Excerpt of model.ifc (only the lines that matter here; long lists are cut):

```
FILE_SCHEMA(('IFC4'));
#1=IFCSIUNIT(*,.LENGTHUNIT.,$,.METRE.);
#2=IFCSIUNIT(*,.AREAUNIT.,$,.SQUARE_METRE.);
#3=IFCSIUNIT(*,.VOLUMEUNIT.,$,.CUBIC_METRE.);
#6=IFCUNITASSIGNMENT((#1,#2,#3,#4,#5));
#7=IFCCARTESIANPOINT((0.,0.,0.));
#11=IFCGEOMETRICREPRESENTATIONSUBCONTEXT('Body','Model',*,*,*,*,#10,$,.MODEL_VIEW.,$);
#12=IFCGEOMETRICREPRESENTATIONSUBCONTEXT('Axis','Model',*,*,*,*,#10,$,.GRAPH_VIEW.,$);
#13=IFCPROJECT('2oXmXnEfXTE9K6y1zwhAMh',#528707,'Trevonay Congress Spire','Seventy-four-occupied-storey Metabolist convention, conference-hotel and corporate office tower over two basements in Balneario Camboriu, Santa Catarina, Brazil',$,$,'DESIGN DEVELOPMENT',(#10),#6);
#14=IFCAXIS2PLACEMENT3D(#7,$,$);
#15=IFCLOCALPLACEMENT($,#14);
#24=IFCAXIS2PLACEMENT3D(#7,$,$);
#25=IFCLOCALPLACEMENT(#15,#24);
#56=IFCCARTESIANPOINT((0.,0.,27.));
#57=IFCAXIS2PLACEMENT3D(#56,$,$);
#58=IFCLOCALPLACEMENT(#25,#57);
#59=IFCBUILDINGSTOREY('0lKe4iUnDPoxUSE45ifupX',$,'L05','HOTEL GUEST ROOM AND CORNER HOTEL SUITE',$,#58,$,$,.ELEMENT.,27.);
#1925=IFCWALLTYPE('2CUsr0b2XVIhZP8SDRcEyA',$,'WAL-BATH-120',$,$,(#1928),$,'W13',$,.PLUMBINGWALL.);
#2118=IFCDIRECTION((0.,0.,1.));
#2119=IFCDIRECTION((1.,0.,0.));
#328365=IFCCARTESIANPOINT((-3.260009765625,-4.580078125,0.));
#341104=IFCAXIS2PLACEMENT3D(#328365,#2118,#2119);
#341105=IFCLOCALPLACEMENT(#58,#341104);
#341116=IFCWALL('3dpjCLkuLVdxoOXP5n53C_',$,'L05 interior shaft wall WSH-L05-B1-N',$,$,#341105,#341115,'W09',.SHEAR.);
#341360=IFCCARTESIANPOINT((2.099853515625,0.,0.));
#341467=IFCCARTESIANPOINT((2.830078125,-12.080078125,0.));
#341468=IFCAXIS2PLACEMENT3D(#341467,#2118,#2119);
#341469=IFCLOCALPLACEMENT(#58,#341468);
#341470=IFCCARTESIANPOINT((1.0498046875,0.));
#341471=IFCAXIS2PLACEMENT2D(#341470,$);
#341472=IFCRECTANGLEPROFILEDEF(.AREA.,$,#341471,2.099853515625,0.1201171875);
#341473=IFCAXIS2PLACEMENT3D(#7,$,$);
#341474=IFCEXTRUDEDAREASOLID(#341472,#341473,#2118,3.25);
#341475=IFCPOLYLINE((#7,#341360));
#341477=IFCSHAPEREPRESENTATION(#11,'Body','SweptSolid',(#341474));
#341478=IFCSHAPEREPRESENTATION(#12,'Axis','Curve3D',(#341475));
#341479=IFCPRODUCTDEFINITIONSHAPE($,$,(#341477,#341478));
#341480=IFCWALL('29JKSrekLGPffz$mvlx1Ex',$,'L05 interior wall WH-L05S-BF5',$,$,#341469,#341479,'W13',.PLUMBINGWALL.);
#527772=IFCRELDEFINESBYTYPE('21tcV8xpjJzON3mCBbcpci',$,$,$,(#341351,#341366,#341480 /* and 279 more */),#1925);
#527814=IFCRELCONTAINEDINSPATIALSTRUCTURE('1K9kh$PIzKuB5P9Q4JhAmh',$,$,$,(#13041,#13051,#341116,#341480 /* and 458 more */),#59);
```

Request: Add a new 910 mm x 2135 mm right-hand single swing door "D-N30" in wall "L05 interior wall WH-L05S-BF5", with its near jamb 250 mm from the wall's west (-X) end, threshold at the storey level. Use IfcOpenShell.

```python
import numpy as np
import ifcopenshell
import ifcopenshell.api.feature
import ifcopenshell.api.geometry
import ifcopenshell.api.root
import ifcopenshell.api.spatial
import ifcopenshell.geom
import ifcopenshell.util.element
import ifcopenshell.util.placement
import ifcopenshell.util.representation
import ifcopenshell.util.shape
import ifcopenshell.util.unit

model = ifcopenshell.open("model.ifc")
unit_scale = ifcopenshell.util.unit.calculate_unit_scale(model)
settings = ifcopenshell.geom.settings()


def volume(element):
    """Net volume in cubic metres, openings subtracted."""
    shape = ifcopenshell.geom.create_shape(settings, element)
    return ifcopenshell.util.shape.get_volume(shape.geometry)


wall = model.by_guid("29JKSrekLGPffz$mvlx1Ex")
storey = ifcopenshell.util.element.get_container(wall, ifc_class="IfcBuildingStorey")
context = ifcopenshell.util.representation.get_context(model, "Model", "Body", "MODEL_VIEW")
before = volume(wall)

width, height, from_end, sill = 0.91, 2.135, 0.25, 0.0  # metres

# The wall runs along its own X axis, and the end named is its -X end.
wall_shape = ifcopenshell.geom.create_shape(settings, wall)
x, y, z = ifcopenshell.util.shape.get_vertices(wall_shape.geometry).T
start = x.min() + from_end
face, thickness = float(y.min()), float(y.max() - y.min())
wall_matrix = ifcopenshell.util.placement.get_local_placement(wall.ObjectPlacement)
level = ifcopenshell.util.placement.get_local_placement(storey.ObjectPlacement)[2, 3]


def in_wall(x, y):
    """Placement at x, y metres in the wall's axes, at sill height."""
    matrix = wall_matrix.copy()
    matrix[:, 3] = wall_matrix @ np.array([x / unit_scale, y / unit_scale, 0.0, 1.0])
    matrix[2, 3] = level + sill / unit_scale
    return matrix


# Opening: a box that overshoots both wall faces by 50 mm.
opening = ifcopenshell.api.root.create_entity(model, ifc_class="IfcOpeningElement", predefined_type="OPENING")
box = ifcopenshell.api.geometry.add_wall_representation(
    model, context=context, length=width, height=height, thickness=thickness + 0.1
)
ifcopenshell.api.geometry.assign_representation(model, product=opening, representation=box)
ifcopenshell.api.geometry.edit_object_placement(model, product=opening, matrix=in_wall(start, face - 0.05), is_si=False)
ifcopenshell.api.feature.add_feature(model, feature=opening, element=wall)

door = ifcopenshell.api.root.create_entity(model, ifc_class="IfcDoor", name="D-N30", predefined_type="DOOR")
door.OverallWidth, door.OverallHeight = width / unit_scale, height / unit_scale
door.OperationType = "SINGLE_SWING_RIGHT"
body = ifcopenshell.api.geometry.add_door_representation(
    model,
    context=context,
    overall_width=door.OverallWidth,
    overall_height=door.OverallHeight,
    operation_type="SINGLE_SWING_RIGHT",
    lining_properties={"LiningDepth": thickness / unit_scale, "ThresholdDepth": thickness / unit_scale},
)
ifcopenshell.api.geometry.assign_representation(model, product=door, representation=body)
ifcopenshell.api.spatial.assign_container(model, products=[door], relating_structure=storey)
ifcopenshell.api.feature.add_filling(model, opening=opening, element=door)

# The lining spans the wall, so the door starts at the wall face.
ifcopenshell.api.geometry.edit_object_placement(model, product=door, matrix=in_wall(start, face), is_si=False)

after = volume(wall)

print(f"wall volume {before:.3f} -> {after:.3f} m3")

model.write("model-out.ifc")
```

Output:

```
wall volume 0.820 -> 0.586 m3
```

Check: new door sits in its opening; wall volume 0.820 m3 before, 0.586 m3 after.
